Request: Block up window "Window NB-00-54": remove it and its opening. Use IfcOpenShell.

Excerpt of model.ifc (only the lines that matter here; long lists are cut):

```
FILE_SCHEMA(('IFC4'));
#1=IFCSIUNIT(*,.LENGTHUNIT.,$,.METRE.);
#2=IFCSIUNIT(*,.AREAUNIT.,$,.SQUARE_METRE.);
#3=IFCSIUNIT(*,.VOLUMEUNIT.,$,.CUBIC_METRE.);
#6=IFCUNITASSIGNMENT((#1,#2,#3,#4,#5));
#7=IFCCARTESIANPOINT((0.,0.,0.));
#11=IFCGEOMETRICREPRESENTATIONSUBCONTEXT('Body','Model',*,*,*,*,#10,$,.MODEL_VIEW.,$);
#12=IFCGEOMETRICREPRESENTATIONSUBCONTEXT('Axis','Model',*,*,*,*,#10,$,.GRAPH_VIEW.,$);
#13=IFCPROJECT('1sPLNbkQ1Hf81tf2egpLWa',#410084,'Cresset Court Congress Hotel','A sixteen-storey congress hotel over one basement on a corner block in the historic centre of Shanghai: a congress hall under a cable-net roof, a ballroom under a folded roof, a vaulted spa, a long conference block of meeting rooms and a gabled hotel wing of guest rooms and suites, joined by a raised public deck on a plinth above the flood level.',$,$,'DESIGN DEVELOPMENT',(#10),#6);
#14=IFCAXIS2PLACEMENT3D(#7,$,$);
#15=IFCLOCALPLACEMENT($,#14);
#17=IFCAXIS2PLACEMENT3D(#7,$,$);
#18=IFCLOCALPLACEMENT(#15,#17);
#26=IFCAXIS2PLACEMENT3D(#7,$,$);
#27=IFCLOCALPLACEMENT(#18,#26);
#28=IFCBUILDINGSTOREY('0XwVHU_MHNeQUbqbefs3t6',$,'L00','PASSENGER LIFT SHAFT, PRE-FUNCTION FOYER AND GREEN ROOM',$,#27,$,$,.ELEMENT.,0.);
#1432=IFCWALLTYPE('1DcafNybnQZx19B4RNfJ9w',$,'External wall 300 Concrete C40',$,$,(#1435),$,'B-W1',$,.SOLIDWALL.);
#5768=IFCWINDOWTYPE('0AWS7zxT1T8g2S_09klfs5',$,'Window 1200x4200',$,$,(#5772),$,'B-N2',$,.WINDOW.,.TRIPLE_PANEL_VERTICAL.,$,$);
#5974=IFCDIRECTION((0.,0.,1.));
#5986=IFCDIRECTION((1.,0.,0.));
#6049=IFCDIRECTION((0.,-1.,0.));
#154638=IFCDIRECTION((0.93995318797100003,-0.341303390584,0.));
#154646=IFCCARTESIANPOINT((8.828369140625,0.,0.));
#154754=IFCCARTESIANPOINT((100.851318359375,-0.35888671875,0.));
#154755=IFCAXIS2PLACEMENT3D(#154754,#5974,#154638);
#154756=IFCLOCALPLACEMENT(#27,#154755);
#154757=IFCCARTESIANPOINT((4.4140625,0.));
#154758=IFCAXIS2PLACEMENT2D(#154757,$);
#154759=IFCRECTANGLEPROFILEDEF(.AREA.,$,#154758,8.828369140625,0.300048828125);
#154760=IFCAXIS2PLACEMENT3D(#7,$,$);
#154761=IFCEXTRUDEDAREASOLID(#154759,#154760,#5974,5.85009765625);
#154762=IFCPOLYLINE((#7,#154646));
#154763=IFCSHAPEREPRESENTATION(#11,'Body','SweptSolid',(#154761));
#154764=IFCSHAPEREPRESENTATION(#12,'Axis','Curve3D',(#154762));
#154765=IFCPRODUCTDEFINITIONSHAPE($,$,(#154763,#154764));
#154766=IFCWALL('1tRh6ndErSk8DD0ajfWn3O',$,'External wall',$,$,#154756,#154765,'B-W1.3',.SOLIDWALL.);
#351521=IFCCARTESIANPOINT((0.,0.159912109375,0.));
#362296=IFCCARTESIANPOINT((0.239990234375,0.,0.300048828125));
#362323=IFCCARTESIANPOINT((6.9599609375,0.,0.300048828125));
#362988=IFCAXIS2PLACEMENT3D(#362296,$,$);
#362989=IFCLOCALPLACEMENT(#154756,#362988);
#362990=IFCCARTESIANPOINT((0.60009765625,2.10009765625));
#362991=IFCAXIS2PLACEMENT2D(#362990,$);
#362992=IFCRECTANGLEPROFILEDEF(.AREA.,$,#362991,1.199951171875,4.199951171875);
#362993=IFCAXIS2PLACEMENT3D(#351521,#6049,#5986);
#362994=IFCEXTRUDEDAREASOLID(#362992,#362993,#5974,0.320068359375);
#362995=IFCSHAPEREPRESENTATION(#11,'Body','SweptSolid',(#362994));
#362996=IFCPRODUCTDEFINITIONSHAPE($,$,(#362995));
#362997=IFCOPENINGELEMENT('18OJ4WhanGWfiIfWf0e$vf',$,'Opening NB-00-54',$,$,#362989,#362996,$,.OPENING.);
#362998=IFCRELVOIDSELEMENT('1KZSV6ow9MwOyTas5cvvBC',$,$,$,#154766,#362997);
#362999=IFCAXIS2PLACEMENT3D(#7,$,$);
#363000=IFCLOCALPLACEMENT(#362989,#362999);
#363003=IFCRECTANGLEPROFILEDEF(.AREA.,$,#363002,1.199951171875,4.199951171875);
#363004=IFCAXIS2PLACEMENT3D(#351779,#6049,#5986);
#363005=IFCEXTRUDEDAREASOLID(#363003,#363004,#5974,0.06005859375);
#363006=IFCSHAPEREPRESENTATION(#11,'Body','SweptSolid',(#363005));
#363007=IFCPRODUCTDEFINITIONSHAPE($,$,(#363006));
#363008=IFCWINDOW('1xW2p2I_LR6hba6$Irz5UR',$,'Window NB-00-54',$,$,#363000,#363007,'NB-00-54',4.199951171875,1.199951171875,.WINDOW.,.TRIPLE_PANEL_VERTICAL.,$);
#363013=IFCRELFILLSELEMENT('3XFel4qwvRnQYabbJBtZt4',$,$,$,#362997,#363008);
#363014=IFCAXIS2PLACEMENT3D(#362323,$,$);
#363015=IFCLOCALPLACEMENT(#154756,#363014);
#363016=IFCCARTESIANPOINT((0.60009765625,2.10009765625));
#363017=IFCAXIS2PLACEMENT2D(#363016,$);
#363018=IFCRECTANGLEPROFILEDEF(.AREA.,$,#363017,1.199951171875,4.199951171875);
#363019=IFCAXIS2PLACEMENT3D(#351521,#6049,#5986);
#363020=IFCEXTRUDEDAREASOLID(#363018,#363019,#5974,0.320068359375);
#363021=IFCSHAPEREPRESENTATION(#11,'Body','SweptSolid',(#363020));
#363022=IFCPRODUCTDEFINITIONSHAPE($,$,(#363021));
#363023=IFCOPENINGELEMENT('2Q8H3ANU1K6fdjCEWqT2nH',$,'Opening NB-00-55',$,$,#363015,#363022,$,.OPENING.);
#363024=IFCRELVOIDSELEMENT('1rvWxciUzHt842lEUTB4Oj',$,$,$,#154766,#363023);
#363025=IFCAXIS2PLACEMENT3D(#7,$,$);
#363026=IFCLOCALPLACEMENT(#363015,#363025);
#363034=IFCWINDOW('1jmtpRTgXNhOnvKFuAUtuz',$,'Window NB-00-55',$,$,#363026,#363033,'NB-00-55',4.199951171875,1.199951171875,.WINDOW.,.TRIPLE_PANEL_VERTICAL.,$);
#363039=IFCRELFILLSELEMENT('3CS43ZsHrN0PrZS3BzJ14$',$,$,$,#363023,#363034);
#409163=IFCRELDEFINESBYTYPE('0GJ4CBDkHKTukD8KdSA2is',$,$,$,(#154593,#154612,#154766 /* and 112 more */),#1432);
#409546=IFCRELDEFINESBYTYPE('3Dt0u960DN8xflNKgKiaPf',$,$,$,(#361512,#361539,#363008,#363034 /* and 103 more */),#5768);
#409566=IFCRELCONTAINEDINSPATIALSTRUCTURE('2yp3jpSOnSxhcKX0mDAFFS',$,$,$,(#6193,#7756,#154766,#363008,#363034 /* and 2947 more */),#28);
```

```python
import ifcopenshell
import ifcopenshell.api.feature
import ifcopenshell.api.root
import ifcopenshell.geom
import ifcopenshell.util.shape

model = ifcopenshell.open("model.ifc")
settings = ifcopenshell.geom.settings()


def volume(element):
    """Net volume in cubic metres, openings subtracted."""
    shape = ifcopenshell.geom.create_shape(settings, element)
    return ifcopenshell.util.shape.get_volume(shape.geometry)


window = model.by_guid("1xW2p2I_LR6hba6$Irz5UR")
opening = window.FillsVoids[0].RelatingOpeningElement
wall = opening.VoidsElements[0].RelatingBuildingElement
before = volume(wall)

ifcopenshell.api.root.remove_product(model, product=window)
ifcopenshell.api.feature.remove_feature(model, feature=opening)

after = volume(wall)

print(f"wall volume {before:.3f} -> {after:.3f} m3")

model.write("model_v2.ifc")
```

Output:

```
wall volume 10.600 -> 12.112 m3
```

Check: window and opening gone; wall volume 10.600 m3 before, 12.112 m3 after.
